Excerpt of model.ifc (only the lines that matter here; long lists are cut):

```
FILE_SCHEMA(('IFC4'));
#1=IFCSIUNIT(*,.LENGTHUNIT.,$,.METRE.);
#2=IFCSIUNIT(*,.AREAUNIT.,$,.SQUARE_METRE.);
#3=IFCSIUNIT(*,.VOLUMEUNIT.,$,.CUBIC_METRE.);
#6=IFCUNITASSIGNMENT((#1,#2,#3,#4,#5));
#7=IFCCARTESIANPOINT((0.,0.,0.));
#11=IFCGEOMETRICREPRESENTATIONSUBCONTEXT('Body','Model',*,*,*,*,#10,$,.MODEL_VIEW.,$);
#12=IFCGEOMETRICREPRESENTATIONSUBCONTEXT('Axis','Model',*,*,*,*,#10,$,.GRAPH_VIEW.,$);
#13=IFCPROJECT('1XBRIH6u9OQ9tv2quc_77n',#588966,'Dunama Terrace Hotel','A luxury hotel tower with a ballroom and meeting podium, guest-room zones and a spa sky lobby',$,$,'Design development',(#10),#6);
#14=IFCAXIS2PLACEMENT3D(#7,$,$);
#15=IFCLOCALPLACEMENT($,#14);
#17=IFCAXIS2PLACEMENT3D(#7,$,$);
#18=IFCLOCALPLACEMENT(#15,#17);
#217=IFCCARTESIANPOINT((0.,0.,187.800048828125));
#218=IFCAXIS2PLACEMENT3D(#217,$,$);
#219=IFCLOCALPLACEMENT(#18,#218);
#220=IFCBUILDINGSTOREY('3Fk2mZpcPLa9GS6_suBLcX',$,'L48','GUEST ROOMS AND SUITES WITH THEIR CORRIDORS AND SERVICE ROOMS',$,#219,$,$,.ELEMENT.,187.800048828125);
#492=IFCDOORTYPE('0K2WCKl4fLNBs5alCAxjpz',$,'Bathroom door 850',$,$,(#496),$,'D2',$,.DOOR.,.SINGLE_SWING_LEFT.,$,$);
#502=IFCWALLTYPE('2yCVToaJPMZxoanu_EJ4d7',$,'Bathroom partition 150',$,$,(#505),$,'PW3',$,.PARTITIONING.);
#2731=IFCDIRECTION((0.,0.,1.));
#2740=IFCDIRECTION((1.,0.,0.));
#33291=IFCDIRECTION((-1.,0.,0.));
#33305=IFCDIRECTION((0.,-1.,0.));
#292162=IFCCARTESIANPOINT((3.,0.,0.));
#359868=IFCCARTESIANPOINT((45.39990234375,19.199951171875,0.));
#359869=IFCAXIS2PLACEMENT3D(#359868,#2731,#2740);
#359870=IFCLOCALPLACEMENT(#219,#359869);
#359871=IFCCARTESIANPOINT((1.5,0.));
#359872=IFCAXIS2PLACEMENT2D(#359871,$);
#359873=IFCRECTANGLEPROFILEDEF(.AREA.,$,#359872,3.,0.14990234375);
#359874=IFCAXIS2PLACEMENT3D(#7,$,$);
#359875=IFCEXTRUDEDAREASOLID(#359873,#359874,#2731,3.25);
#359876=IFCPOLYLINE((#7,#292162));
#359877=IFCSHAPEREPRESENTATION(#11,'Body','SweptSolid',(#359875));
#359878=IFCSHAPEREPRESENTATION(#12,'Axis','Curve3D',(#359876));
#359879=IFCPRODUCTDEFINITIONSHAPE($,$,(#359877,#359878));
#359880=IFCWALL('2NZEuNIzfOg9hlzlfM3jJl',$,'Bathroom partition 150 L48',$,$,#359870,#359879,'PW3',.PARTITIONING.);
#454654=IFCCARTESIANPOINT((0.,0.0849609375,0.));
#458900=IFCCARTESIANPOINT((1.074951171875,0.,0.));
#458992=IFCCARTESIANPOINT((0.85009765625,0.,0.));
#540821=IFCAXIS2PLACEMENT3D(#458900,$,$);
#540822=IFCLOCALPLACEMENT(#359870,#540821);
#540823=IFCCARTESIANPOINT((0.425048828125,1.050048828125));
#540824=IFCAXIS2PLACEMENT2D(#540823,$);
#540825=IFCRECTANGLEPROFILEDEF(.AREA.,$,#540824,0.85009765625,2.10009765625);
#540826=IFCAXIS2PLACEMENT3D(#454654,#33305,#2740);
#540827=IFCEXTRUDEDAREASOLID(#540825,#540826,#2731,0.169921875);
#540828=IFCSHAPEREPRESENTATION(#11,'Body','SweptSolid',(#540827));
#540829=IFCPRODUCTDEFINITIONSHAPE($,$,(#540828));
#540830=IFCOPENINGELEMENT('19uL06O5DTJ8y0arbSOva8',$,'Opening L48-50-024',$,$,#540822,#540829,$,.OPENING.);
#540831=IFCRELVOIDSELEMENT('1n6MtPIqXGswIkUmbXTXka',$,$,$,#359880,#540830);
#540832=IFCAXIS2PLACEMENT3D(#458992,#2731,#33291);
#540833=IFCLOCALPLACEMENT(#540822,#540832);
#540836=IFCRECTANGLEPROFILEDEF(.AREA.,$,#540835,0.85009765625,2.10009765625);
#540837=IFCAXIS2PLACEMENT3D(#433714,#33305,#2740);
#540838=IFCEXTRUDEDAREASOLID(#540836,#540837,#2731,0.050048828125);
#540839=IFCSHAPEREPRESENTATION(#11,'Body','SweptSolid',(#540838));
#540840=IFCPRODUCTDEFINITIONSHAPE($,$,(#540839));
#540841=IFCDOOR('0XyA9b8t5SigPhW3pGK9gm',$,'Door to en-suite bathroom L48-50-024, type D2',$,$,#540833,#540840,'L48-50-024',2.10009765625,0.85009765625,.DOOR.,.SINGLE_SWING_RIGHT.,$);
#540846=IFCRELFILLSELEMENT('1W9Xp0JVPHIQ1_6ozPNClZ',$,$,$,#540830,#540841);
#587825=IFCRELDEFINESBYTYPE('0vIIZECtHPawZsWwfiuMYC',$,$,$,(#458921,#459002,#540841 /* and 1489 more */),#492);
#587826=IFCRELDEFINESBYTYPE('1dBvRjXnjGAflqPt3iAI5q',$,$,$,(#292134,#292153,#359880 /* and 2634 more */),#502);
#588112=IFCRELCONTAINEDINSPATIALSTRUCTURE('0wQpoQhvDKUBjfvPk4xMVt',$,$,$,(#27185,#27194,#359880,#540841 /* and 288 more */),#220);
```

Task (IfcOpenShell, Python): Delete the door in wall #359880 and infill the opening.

```python
import ifcopenshell
import ifcopenshell.api.feature
import ifcopenshell.api.root
import ifcopenshell.geom
import ifcopenshell.util.shape

model = ifcopenshell.open("model.ifc")
settings = ifcopenshell.geom.settings()


def volume(element):
    """Net volume in cubic metres, openings subtracted."""
    shape = ifcopenshell.geom.create_shape(settings, element)
    return ifcopenshell.util.shape.get_volume(shape.geometry)


door = model.by_guid("0XyA9b8t5SigPhW3pGK9gm")
opening = door.FillsVoids[0].RelatingOpeningElement
wall = opening.VoidsElements[0].RelatingBuildingElement
before = volume(wall)

ifcopenshell.api.root.remove_product(model, product=door)
ifcopenshell.api.feature.remove_feature(model, feature=opening)

after = volume(wall)

print(f"wall volume {before:.3f} -> {after:.3f} m3")

model.write("model_updated.ifc")
```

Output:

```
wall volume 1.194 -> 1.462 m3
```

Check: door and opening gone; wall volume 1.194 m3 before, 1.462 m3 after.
